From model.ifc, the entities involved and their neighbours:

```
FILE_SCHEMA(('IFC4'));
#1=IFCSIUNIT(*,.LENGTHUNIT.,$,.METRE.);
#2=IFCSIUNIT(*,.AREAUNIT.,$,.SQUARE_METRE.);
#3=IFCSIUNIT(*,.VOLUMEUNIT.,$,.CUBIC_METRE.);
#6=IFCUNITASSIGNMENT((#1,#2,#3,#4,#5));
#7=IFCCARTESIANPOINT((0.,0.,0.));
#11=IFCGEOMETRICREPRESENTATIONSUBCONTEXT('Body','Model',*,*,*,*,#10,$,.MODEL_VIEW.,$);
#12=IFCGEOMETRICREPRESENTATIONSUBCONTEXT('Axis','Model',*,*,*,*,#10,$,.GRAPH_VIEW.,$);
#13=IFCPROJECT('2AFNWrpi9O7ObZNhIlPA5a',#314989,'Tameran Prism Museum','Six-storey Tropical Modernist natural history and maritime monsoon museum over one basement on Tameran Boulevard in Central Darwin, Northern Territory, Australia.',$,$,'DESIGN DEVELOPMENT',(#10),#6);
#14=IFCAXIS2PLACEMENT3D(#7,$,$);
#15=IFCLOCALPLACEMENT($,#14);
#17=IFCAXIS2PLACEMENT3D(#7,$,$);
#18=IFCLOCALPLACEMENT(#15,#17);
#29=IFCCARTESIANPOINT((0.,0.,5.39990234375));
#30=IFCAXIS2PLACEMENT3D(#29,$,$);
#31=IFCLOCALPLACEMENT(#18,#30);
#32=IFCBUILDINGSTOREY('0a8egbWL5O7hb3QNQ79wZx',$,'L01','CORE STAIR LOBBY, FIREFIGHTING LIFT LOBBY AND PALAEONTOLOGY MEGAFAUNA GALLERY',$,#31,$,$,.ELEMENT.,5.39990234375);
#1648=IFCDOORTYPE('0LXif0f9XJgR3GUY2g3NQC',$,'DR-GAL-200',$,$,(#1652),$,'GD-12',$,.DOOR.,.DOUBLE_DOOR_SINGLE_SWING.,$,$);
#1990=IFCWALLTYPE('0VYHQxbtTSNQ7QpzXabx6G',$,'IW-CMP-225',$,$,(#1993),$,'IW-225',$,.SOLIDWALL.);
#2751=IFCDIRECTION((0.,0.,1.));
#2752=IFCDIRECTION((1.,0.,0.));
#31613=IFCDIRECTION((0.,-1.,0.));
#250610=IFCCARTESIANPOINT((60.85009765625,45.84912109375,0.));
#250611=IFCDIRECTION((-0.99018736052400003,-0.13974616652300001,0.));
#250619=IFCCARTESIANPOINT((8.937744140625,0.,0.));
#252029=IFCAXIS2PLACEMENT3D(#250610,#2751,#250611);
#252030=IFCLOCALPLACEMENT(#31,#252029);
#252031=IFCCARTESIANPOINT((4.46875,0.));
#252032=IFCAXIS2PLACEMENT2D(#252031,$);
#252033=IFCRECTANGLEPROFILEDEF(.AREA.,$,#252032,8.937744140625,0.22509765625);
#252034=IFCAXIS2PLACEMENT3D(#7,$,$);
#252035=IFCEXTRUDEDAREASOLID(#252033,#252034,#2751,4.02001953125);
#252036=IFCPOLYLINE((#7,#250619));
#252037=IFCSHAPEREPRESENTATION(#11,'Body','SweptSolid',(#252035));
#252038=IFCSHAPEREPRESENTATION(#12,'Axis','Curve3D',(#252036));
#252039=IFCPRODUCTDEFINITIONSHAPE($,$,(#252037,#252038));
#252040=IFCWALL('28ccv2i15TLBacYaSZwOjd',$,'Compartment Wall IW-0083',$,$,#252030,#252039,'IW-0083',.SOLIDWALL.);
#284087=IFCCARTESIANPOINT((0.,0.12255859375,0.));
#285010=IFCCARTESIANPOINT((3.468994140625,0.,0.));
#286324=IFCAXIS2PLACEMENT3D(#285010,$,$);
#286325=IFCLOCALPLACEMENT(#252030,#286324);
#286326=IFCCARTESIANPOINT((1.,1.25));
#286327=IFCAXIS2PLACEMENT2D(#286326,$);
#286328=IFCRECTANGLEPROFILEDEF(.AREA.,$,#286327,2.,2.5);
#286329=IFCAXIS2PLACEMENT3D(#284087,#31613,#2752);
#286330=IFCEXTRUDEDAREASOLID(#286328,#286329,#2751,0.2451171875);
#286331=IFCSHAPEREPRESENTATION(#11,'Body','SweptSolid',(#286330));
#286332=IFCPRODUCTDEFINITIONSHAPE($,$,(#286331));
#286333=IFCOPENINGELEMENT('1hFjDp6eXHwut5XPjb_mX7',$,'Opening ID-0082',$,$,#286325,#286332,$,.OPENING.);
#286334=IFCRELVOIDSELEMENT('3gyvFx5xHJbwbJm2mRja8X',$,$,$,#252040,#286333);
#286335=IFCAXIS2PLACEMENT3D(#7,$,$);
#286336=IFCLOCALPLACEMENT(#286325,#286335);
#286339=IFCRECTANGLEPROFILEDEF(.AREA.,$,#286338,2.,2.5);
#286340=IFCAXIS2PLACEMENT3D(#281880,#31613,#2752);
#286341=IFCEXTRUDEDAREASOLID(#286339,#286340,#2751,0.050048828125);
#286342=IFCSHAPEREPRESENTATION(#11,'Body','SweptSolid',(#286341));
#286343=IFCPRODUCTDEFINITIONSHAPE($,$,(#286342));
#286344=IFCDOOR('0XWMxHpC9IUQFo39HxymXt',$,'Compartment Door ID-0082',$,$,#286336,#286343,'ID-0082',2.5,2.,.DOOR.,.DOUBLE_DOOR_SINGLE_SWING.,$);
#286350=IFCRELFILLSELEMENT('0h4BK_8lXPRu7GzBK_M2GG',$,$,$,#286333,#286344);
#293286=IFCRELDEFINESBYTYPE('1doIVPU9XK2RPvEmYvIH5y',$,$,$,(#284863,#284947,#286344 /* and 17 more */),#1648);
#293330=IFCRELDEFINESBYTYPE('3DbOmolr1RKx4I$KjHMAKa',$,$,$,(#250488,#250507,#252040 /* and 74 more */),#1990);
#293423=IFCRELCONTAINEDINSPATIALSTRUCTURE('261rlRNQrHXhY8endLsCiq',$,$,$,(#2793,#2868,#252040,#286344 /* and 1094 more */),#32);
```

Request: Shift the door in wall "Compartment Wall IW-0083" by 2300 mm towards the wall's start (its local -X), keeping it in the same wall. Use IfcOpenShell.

```python
import ifcopenshell
import ifcopenshell.api.geometry
import ifcopenshell.util.placement

model = ifcopenshell.open("model.ifc")

door = model.by_id(286344)
opening = door.FillsVoids[0].RelatingOpeningElement
wall = opening.VoidsElements[0].RelatingBuildingElement

wall_matrix = ifcopenshell.util.placement.get_local_placement(wall.ObjectPlacement)
shift = wall_matrix[:3, 0] * -2.3
before = ifcopenshell.util.placement.get_local_placement(door.ObjectPlacement)[:3, 3].copy()

# The door is placed relative to its opening, so it follows when the opening moves.
matrix = ifcopenshell.util.placement.get_local_placement(opening.ObjectPlacement)
matrix[:3, 3] += shift
ifcopenshell.api.geometry.edit_object_placement(
    model, product=opening, matrix=matrix, is_si=False, should_transform_children=True
)

after = ifcopenshell.util.placement.get_local_placement(door.ObjectPlacement)[:3, 3]
print("door moved by", (after - before).round(3) + 0.0)

model.write("model-out.ifc")
```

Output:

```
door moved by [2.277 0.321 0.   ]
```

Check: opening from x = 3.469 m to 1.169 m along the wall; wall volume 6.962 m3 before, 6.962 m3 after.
